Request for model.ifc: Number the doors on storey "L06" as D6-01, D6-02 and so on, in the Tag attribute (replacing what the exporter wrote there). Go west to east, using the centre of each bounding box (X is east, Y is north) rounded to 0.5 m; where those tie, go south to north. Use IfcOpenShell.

First a look at what the model holds.

```python
import ifcopenshell
import ifcopenshell.util.element
import ifcopenshell.util.placement

model = ifcopenshell.open("model.ifc")
print(model.schema)
storey = next(s for s in model.by_type("IfcBuildingStorey") if s.Name == "L06")
doors = [e for e in ifcopenshell.util.element.get_decomposition(storey) if e.is_a("IfcDoor")]
for e in sorted(doors, key=lambda e: e.id()):
    origin = ifcopenshell.util.placement.get_local_placement(e.ObjectPlacement)[:3, 3]
    print(e.id(), e.Tag, e.Name, origin.round(2) + 0.0, sep=" | ")
```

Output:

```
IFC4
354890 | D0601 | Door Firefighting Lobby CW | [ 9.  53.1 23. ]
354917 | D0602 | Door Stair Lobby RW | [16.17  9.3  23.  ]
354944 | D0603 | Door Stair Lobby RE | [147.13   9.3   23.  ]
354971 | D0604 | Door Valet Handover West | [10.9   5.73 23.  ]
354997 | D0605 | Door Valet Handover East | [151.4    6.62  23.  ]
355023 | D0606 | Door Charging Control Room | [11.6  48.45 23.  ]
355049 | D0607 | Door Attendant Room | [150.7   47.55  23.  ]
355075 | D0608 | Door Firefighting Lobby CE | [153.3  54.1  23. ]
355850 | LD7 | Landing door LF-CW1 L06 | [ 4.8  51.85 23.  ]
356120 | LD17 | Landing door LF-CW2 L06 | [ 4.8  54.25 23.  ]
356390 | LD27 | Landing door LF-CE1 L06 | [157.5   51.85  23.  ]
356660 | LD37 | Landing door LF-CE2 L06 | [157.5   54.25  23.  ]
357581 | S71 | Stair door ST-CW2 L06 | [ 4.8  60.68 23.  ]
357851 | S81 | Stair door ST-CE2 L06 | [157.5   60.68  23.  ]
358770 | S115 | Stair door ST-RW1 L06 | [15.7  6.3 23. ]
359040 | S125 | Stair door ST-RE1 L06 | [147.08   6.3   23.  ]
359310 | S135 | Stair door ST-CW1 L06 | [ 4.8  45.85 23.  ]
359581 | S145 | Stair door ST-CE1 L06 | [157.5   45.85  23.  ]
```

```python
import ifcopenshell
import ifcopenshell.geom
import ifcopenshell.util.element
import ifcopenshell.util.shape

model = ifcopenshell.open("model.ifc")
settings = ifcopenshell.geom.settings()
settings.set("use-world-coords", True)


def centre(element):
    shape = ifcopenshell.geom.create_shape(settings, element)
    return ifcopenshell.util.shape.get_bbox_centroid(shape.geometry)


storey = next(s for s in model.by_type("IfcBuildingStorey") if s.Name == "L06")
doors = [e for e in ifcopenshell.util.element.get_decomposition(storey) if e.is_a("IfcDoor")]

# Insertion points can sit at a corner or the storey origin, so sort by the geometry (in metres).
centres = {e: centre(e) for e in doors}
doors.sort(key=lambda e: (round(centres[e][0] / 0.5), centres[e][1]))

for i, e in enumerate(doors, start=1):
    number = f"D6-{i:02d}"
    e.Tag = number
    print(e.id(), number)

model.write("model_rev.ifc")
```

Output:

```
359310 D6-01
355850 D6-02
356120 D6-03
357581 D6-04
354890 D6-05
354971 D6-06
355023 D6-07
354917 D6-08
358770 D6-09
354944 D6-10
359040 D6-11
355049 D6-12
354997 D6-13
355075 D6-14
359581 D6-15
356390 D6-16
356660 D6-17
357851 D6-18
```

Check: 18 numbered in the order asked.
